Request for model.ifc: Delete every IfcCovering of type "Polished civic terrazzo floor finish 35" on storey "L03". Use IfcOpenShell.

First a look at what the model holds.

```python
import ifcopenshell
import ifcopenshell.util.element

model = ifcopenshell.open("model.ifc")
print(model.schema)
storey = next(s for s in model.by_type("IfcBuildingStorey") if s.Name == "L03")
coverings = [e for e in ifcopenshell.util.element.get_decomposition(storey) if e.is_a("IfcCovering")]
seen = {}
for e in coverings:
    element_type = ifcopenshell.util.element.get_type(e)
    name = element_type.Name if element_type not in (None, e) else None
    seen[name] = seen.get(name, 0) + 1
for name, count in sorted(seen.items(), key=str):
    print(count, "x", name)
```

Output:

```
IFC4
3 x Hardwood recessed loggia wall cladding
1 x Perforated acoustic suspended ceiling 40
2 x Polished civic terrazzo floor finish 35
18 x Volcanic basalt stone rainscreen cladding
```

```python
import ifcopenshell
import ifcopenshell.api.root
import ifcopenshell.util.element

model = ifcopenshell.open("model.ifc")

storey = next(s for s in model.by_type("IfcBuildingStorey") if s.Name == "L03")
coverings = [e for e in ifcopenshell.util.element.get_decomposition(storey) if e.is_a("IfcCovering")]
targets = [e for e in coverings if (t := ifcopenshell.util.element.get_type(e)) not in (None, e) and t.Name == "Polished civic terrazzo floor finish 35"]

for e in targets:
    ifcopenshell.api.root.remove_product(model, product=e)
print(len(targets), "removed")

model.write("model_rev.ifc")
```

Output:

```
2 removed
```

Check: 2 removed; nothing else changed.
